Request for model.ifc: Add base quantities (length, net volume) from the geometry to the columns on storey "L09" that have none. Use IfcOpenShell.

First a look at what the model holds.

```python
import ifcopenshell
import ifcopenshell.util.element
import ifcopenshell.util.unit

model = ifcopenshell.open("model.ifc")
print(model.schema)
for unit_type in ("LENGTHUNIT", "AREAUNIT", "VOLUMEUNIT"):
    print(unit_type, ifcopenshell.util.unit.calculate_unit_scale(model, unit_type))
storey = next(s for s in model.by_type("IfcBuildingStorey") if s.Name == "L09")
columns = [e for e in ifcopenshell.util.element.get_decomposition(storey) if e.is_a("IfcColumn")]
for e in sorted(columns, key=lambda e: e.id()):
    print(e.id(), e.is_a(), e.Name, list(ifcopenshell.util.element.get_psets(e, qtos_only=True)), sep=" | ")
```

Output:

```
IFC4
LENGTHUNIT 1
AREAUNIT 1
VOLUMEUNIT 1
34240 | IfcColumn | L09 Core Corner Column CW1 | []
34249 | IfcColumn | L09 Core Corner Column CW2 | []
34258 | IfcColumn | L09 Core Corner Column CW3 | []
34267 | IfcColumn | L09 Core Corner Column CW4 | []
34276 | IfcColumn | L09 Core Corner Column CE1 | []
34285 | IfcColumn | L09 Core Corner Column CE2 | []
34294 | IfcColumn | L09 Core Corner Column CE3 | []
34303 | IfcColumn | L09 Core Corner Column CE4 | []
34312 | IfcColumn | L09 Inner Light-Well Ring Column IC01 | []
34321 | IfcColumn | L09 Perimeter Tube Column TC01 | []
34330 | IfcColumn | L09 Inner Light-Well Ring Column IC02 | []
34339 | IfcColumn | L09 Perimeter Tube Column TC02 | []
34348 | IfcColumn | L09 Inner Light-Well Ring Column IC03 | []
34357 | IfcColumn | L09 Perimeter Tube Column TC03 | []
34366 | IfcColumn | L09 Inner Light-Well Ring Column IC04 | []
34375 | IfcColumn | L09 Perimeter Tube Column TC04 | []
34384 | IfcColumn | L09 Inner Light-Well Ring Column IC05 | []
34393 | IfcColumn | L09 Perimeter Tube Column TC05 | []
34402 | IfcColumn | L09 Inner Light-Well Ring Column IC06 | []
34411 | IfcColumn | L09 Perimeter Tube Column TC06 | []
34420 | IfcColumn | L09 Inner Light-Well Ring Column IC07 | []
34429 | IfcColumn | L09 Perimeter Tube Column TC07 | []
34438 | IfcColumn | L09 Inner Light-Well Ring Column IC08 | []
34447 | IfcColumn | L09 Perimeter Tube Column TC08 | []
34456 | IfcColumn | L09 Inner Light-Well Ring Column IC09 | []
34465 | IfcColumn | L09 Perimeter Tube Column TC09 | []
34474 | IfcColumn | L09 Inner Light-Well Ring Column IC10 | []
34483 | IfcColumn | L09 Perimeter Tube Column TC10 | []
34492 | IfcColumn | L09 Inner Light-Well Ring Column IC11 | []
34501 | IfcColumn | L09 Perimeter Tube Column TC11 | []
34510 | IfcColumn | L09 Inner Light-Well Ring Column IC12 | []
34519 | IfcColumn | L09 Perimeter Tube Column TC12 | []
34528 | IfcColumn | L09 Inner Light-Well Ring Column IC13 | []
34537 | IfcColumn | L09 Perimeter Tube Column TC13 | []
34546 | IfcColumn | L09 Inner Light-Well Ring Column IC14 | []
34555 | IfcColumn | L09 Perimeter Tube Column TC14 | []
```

```python
import ifcopenshell
import ifcopenshell.api.pset
import ifcopenshell.geom
import ifcopenshell.util.element
import ifcopenshell.util.shape
import ifcopenshell.util.unit

model = ifcopenshell.open("model.ifc")
unit_scale = ifcopenshell.util.unit.calculate_unit_scale(model)
volume_scale = ifcopenshell.util.unit.calculate_unit_scale(model, "VOLUMEUNIT")
settings = ifcopenshell.geom.settings()

storey = next(s for s in model.by_type("IfcBuildingStorey") if s.Name == "L09")
columns = [e for e in ifcopenshell.util.element.get_decomposition(storey) if e.is_a("IfcColumn")]

for e in sorted(columns, key=lambda e: e.id()):
    if ifcopenshell.util.element.get_psets(e, qtos_only=True, should_inherit=False):
        continue
    # Geometry comes back in metres, in the element's own axes.
    shape = ifcopenshell.geom.create_shape(settings, e)
    values = {
        "Length": ifcopenshell.util.shape.get_z(shape.geometry) / unit_scale,
        "NetVolume": ifcopenshell.util.shape.get_volume(shape.geometry) / volume_scale,
    }
    qto = ifcopenshell.api.pset.add_qto(model, product=e, name="Qto_ColumnBaseQuantities")
    ifcopenshell.api.pset.edit_qto(model, qto=qto, properties=values)
    print(e.id(), {k: round(v, 3) for k, v in values.items()})

model.write("model_updated.ifc")
```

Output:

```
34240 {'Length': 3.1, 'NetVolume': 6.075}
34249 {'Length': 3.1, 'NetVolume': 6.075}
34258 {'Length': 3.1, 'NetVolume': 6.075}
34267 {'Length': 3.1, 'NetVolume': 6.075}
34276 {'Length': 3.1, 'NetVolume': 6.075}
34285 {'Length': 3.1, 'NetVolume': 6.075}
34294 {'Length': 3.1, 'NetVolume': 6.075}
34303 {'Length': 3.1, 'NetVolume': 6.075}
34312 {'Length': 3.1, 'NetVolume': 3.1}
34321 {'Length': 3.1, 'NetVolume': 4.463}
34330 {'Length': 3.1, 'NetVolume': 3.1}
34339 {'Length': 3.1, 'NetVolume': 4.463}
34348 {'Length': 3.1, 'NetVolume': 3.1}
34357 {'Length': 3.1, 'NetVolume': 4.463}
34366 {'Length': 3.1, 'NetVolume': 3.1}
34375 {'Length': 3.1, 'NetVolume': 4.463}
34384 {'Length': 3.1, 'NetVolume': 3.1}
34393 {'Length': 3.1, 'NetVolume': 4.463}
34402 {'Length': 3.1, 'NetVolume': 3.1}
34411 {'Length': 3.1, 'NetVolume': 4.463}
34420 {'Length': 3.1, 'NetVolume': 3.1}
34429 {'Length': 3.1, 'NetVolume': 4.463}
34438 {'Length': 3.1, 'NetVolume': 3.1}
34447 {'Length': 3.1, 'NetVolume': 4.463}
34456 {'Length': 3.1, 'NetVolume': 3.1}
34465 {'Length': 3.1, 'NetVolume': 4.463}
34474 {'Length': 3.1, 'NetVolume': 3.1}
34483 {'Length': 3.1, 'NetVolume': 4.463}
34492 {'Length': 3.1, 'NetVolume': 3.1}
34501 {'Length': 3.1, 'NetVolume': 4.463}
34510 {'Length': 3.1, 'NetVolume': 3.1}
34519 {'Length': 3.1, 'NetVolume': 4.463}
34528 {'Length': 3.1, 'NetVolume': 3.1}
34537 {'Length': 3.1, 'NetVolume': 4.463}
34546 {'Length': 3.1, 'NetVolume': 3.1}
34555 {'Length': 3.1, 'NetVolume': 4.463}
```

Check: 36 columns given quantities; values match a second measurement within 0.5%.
